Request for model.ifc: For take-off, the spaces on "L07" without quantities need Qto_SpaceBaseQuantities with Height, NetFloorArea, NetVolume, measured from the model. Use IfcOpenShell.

First a look at what the model holds.

```python
import ifcopenshell
import ifcopenshell.util.element
import ifcopenshell.util.unit

model = ifcopenshell.open("model.ifc")
print(model.schema)
for unit_type in ("LENGTHUNIT", "AREAUNIT", "VOLUMEUNIT"):
    print(unit_type, ifcopenshell.util.unit.calculate_unit_scale(model, unit_type))
storey = next(s for s in model.by_type("IfcBuildingStorey") if s.Name == "L07")
spaces = [e for e in ifcopenshell.util.element.get_decomposition(storey) if e.is_a("IfcSpace")]
for e in sorted(spaces, key=lambda e: e.id()):
    print(e.id(), e.is_a(), e.Name, list(ifcopenshell.util.element.get_psets(e, qtos_only=True)), sep=" | ")
```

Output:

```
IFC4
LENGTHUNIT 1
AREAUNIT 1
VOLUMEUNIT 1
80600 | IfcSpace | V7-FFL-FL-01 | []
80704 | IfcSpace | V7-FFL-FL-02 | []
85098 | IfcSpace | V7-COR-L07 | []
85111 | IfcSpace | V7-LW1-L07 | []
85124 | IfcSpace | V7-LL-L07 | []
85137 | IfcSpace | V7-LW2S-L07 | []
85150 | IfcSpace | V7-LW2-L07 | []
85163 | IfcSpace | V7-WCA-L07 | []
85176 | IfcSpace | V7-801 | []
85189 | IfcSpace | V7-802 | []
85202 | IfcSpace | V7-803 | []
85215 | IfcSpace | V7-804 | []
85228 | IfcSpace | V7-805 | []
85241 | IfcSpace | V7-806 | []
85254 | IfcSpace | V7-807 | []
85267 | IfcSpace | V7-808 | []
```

```python
import ifcopenshell
import ifcopenshell.api.pset
import ifcopenshell.geom
import ifcopenshell.util.element
import ifcopenshell.util.shape
import ifcopenshell.util.unit

model = ifcopenshell.open("model.ifc")
unit_scale = ifcopenshell.util.unit.calculate_unit_scale(model)
area_scale = ifcopenshell.util.unit.calculate_unit_scale(model, "AREAUNIT")
volume_scale = ifcopenshell.util.unit.calculate_unit_scale(model, "VOLUMEUNIT")
settings = ifcopenshell.geom.settings()

storey = next(s for s in model.by_type("IfcBuildingStorey") if s.Name == "L07")
spaces = [e for e in ifcopenshell.util.element.get_decomposition(storey) if e.is_a("IfcSpace")]

for e in sorted(spaces, key=lambda e: e.id()):
    if ifcopenshell.util.element.get_psets(e, qtos_only=True, should_inherit=False):
        continue
    # Geometry comes back in metres, in the element's own axes.
    shape = ifcopenshell.geom.create_shape(settings, e)
    values = {
        "Height": ifcopenshell.util.shape.get_z(shape.geometry) / unit_scale,
        "NetFloorArea": ifcopenshell.util.shape.get_footprint_area(shape.geometry) / area_scale,
        "NetVolume": ifcopenshell.util.shape.get_volume(shape.geometry) / volume_scale,
    }
    qto = ifcopenshell.api.pset.add_qto(model, product=e, name="Qto_SpaceBaseQuantities")
    ifcopenshell.api.pset.edit_qto(model, qto=qto, properties=values)
    print(e.id(), {k: round(v, 3) for k, v in values.items()})

model.write("model_edited.ifc")
```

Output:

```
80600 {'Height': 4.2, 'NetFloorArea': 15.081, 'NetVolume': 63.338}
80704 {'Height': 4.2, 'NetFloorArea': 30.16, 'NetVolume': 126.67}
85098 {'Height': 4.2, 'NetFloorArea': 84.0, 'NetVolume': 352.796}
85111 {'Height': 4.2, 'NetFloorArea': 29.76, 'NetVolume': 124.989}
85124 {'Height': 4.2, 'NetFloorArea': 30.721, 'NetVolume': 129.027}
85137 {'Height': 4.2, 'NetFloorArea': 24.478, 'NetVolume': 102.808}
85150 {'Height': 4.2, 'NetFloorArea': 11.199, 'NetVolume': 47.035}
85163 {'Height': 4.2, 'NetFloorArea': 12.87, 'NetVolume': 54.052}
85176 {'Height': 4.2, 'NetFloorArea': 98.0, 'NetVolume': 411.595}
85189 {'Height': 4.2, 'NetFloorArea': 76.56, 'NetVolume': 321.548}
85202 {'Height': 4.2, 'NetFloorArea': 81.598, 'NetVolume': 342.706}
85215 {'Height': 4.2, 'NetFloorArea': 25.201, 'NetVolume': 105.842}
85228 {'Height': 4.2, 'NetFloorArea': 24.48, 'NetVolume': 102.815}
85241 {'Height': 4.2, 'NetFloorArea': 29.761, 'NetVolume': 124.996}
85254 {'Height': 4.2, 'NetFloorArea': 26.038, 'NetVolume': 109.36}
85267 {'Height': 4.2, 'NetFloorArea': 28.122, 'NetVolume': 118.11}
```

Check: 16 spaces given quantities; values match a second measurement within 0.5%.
